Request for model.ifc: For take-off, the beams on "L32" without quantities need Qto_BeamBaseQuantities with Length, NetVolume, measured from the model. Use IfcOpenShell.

First a look at what the model holds.

```python
import ifcopenshell
import ifcopenshell.util.element
import ifcopenshell.util.unit

model = ifcopenshell.open("model.ifc")
print(model.schema)
for unit_type in ("LENGTHUNIT", "AREAUNIT", "VOLUMEUNIT"):
    print(unit_type, ifcopenshell.util.unit.calculate_unit_scale(model, unit_type))
storey = next(s for s in model.by_type("IfcBuildingStorey") if s.Name == "L32")
beams = [e for e in ifcopenshell.util.element.get_decomposition(storey) if e.is_a("IfcBeam")]
for e in sorted(beams, key=lambda e: e.id()):
    print(e.id(), e.is_a(), e.Name, list(ifcopenshell.util.element.get_psets(e, qtos_only=True)), sep=" | ")
```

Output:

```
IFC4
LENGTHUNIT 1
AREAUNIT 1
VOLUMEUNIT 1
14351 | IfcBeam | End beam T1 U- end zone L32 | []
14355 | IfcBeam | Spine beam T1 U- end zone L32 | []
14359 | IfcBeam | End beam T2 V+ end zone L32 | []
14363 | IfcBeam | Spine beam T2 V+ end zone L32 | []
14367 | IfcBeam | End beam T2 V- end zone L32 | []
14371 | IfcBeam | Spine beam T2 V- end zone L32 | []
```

```python
import ifcopenshell
import ifcopenshell.api.pset
import ifcopenshell.geom
import ifcopenshell.util.element
import ifcopenshell.util.shape
import ifcopenshell.util.unit

model = ifcopenshell.open("model.ifc")
unit_scale = ifcopenshell.util.unit.calculate_unit_scale(model)
volume_scale = ifcopenshell.util.unit.calculate_unit_scale(model, "VOLUMEUNIT")
settings = ifcopenshell.geom.settings()

storey = next(s for s in model.by_type("IfcBuildingStorey") if s.Name == "L32")
beams = [e for e in ifcopenshell.util.element.get_decomposition(storey) if e.is_a("IfcBeam")]

for e in sorted(beams, key=lambda e: e.id()):
    if ifcopenshell.util.element.get_psets(e, qtos_only=True, should_inherit=False):
        continue
    # Geometry comes back in metres, in the element's own axes.
    shape = ifcopenshell.geom.create_shape(settings, e)
    values = {
        "Length": ifcopenshell.util.shape.get_max_xyz(shape.geometry) / unit_scale,
        "NetVolume": ifcopenshell.util.shape.get_volume(shape.geometry) / volume_scale,
    }
    qto = ifcopenshell.api.pset.add_qto(model, product=e, name="Qto_BeamBaseQuantities")
    ifcopenshell.api.pset.edit_qto(model, qto=qto, properties=values)
    print(e.id(), {k: round(v, 3) for k, v in values.items()})

model.write("model-out.ifc")
```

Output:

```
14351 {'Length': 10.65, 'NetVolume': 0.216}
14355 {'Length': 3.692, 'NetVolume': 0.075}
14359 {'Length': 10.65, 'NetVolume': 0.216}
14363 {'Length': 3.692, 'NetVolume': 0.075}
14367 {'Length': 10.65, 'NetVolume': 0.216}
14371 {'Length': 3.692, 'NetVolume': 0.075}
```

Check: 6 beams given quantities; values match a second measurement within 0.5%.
